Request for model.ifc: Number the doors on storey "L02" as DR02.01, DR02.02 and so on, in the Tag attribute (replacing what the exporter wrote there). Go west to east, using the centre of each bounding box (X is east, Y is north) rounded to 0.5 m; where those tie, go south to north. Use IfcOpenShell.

First a look at what the model holds.

```python
import ifcopenshell
import ifcopenshell.util.element
import ifcopenshell.util.placement

model = ifcopenshell.open("model.ifc")
print(model.schema)
storey = next(s for s in model.by_type("IfcBuildingStorey") if s.Name == "L02")
doors = [e for e in ifcopenshell.util.element.get_decomposition(storey) if e.is_a("IfcDoor")]
for e in sorted(doors, key=lambda e: e.id()):
    origin = ifcopenshell.util.placement.get_local_placement(e.ObjectPlacement)[:3, 3]
    print(e.id(), e.Tag, e.Name, origin.round(2) + 0.0, sep=" | ")
```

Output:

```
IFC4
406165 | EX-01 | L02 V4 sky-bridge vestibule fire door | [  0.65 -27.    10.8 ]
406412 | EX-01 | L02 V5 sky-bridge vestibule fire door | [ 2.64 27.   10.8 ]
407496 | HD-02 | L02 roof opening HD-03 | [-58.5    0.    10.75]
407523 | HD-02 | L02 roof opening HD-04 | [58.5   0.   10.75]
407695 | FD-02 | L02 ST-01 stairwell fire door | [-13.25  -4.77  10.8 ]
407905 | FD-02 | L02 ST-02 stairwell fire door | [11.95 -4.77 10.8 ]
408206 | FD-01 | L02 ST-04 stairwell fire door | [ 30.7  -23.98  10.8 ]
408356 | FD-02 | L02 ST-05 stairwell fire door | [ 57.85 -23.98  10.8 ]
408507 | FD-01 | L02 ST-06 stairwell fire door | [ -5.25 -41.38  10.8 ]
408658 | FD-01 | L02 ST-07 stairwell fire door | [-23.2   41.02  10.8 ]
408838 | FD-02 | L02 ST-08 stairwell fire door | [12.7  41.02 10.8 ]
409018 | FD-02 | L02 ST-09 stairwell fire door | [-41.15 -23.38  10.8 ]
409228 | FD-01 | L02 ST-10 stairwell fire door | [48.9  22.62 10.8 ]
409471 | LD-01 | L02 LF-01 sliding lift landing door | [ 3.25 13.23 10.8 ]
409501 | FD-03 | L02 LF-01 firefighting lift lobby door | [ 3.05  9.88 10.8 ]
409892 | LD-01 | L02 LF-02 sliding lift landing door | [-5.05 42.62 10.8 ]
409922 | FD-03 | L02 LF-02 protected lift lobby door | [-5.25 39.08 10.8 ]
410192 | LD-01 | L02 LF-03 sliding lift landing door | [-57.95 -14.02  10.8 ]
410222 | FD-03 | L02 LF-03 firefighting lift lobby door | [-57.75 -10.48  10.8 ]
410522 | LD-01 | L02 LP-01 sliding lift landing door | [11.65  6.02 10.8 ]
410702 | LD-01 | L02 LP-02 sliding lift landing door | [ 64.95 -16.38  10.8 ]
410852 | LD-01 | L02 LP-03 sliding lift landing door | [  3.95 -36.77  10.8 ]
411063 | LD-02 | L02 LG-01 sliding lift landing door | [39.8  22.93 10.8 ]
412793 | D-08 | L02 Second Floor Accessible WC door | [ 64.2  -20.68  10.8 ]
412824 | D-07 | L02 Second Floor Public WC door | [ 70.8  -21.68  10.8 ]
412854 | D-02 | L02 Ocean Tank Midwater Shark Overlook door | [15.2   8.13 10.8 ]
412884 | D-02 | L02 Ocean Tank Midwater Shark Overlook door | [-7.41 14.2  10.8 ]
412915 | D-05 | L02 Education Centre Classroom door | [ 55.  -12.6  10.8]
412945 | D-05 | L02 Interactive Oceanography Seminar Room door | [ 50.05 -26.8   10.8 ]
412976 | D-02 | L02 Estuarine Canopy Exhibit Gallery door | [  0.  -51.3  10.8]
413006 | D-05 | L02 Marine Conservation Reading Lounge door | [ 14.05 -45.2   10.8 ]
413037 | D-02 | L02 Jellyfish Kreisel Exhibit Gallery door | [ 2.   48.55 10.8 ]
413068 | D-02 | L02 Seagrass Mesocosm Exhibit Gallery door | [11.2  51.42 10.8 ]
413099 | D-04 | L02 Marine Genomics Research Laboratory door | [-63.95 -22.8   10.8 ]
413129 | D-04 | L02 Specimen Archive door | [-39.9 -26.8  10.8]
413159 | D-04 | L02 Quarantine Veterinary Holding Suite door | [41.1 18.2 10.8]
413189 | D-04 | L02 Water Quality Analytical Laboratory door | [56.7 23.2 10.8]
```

```python
import ifcopenshell
import ifcopenshell.geom
import ifcopenshell.util.element
import ifcopenshell.util.shape

model = ifcopenshell.open("model.ifc")
settings = ifcopenshell.geom.settings()
settings.set("use-world-coords", True)


def centre(element):
    shape = ifcopenshell.geom.create_shape(settings, element)
    return ifcopenshell.util.shape.get_bbox_centroid(shape.geometry)


storey = next(s for s in model.by_type("IfcBuildingStorey") if s.Name == "L02")
doors = [e for e in ifcopenshell.util.element.get_decomposition(storey) if e.is_a("IfcDoor")]

# Insertion points can sit at a corner or the storey origin, so sort by the geometry (in metres).
centres = {e: centre(e) for e in doors}
doors.sort(key=lambda e: (round(centres[e][0] / 0.5), centres[e][1]))

for i, e in enumerate(doors, start=1):
    number = f"DR02.{i:02d}"
    e.Tag = number
    print(e.id(), number)

model.write("model_edited.ifc")
```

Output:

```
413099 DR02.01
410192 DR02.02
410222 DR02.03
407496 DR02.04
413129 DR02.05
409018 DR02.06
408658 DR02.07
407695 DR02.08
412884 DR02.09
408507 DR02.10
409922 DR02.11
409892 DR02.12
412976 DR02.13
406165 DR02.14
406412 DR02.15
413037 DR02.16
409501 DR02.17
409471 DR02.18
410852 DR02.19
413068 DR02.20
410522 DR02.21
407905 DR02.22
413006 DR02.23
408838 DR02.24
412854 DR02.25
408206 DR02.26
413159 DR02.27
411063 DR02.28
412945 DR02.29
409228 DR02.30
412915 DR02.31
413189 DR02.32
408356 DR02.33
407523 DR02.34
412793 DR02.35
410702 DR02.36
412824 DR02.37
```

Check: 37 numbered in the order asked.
